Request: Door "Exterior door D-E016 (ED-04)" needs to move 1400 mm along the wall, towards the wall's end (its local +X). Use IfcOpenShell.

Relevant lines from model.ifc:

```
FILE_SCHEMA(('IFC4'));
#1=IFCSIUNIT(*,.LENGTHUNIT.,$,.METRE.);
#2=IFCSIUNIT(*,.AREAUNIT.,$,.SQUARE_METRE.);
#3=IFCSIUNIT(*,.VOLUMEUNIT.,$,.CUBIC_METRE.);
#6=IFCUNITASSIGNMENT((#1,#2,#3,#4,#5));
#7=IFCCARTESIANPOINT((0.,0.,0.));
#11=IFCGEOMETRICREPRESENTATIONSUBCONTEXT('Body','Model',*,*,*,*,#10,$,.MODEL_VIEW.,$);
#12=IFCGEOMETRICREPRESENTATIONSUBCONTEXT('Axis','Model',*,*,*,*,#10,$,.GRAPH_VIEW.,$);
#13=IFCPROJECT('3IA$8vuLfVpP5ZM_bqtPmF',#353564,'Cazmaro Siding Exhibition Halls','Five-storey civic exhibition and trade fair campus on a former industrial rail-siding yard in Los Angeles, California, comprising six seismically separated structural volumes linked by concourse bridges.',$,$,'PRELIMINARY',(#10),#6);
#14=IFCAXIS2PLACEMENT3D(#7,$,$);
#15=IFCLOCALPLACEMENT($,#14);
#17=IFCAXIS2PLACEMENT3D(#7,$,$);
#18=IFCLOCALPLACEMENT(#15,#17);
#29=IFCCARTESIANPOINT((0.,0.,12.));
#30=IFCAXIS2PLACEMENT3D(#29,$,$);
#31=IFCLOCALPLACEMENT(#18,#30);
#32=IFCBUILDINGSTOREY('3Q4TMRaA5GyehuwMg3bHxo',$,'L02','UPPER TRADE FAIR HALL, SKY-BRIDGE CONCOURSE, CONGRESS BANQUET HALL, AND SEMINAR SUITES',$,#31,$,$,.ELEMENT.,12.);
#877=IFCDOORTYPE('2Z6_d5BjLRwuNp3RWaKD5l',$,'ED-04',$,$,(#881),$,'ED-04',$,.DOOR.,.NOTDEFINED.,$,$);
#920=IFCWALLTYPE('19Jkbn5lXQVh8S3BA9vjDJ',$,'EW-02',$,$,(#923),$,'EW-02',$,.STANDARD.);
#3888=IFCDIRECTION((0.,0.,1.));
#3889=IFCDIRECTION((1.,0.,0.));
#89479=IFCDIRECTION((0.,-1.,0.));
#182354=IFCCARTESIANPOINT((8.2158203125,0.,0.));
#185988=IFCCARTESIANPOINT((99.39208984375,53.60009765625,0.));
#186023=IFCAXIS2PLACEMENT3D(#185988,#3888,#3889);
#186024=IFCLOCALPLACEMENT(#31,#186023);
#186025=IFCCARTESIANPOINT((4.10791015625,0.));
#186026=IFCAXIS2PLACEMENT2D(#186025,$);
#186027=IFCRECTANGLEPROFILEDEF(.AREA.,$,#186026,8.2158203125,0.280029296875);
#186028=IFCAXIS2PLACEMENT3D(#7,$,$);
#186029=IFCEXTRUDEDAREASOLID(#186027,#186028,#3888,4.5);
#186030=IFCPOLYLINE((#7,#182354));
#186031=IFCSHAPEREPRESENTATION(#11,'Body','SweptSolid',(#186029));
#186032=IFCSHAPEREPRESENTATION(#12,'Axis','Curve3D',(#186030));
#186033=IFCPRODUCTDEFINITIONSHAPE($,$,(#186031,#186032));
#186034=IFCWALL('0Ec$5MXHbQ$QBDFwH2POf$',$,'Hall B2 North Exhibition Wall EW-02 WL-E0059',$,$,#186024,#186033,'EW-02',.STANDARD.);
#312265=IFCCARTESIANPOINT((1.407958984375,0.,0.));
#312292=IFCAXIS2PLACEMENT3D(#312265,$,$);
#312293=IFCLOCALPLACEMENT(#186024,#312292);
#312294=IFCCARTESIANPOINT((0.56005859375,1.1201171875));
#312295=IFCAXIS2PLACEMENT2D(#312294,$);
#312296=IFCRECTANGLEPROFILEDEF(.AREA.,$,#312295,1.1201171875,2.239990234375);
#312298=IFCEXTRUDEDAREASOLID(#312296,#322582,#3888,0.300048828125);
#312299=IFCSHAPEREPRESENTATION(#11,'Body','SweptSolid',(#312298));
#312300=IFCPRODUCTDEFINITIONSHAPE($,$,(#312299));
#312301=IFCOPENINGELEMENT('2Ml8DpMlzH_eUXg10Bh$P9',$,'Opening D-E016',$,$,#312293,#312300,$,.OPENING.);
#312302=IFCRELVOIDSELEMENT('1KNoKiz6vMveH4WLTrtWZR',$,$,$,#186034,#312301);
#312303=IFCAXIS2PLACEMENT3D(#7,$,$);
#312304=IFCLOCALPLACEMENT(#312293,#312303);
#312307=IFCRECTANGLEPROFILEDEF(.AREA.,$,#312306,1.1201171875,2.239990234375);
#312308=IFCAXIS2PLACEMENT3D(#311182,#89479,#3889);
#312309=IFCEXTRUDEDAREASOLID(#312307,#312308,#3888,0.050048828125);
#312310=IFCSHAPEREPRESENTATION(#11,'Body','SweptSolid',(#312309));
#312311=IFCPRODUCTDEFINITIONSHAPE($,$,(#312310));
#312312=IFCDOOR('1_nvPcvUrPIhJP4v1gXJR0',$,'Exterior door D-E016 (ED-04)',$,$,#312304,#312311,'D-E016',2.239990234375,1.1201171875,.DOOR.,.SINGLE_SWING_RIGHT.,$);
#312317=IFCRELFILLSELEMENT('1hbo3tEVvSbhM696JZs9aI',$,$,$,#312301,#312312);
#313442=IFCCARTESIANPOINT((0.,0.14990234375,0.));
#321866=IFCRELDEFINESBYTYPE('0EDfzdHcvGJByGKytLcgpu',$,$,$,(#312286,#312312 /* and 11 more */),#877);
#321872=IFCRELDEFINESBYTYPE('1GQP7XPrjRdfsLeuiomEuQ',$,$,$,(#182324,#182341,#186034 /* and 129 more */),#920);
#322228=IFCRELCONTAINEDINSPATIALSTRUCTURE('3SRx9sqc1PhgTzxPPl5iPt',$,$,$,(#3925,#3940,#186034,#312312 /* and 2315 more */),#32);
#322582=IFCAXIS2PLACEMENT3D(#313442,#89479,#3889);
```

```python
import ifcopenshell
import ifcopenshell.api.geometry
import ifcopenshell.util.placement
import ifcopenshell.util.unit

model = ifcopenshell.open("model.ifc")
unit_scale = ifcopenshell.util.unit.calculate_unit_scale(model)

door = model.by_guid("1_nvPcvUrPIhJP4v1gXJR0")
opening = door.FillsVoids[0].RelatingOpeningElement
wall = opening.VoidsElements[0].RelatingBuildingElement

wall_matrix = ifcopenshell.util.placement.get_local_placement(wall.ObjectPlacement)
shift = wall_matrix[:3, 0] * 1.4 / unit_scale
before = ifcopenshell.util.placement.get_local_placement(door.ObjectPlacement)[:3, 3].copy()

# The door is placed relative to its opening, so it follows when the opening moves.
matrix = ifcopenshell.util.placement.get_local_placement(opening.ObjectPlacement)
matrix[:3, 3] += shift
ifcopenshell.api.geometry.edit_object_placement(
    model, product=opening, matrix=matrix, is_si=False, should_transform_children=True
)

after = ifcopenshell.util.placement.get_local_placement(door.ObjectPlacement)[:3, 3]
print("door moved by", (after - before).round(3) + 0.0)

model.write("model_rev.ifc")
```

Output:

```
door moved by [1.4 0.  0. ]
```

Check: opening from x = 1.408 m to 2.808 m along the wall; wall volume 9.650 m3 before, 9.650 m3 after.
